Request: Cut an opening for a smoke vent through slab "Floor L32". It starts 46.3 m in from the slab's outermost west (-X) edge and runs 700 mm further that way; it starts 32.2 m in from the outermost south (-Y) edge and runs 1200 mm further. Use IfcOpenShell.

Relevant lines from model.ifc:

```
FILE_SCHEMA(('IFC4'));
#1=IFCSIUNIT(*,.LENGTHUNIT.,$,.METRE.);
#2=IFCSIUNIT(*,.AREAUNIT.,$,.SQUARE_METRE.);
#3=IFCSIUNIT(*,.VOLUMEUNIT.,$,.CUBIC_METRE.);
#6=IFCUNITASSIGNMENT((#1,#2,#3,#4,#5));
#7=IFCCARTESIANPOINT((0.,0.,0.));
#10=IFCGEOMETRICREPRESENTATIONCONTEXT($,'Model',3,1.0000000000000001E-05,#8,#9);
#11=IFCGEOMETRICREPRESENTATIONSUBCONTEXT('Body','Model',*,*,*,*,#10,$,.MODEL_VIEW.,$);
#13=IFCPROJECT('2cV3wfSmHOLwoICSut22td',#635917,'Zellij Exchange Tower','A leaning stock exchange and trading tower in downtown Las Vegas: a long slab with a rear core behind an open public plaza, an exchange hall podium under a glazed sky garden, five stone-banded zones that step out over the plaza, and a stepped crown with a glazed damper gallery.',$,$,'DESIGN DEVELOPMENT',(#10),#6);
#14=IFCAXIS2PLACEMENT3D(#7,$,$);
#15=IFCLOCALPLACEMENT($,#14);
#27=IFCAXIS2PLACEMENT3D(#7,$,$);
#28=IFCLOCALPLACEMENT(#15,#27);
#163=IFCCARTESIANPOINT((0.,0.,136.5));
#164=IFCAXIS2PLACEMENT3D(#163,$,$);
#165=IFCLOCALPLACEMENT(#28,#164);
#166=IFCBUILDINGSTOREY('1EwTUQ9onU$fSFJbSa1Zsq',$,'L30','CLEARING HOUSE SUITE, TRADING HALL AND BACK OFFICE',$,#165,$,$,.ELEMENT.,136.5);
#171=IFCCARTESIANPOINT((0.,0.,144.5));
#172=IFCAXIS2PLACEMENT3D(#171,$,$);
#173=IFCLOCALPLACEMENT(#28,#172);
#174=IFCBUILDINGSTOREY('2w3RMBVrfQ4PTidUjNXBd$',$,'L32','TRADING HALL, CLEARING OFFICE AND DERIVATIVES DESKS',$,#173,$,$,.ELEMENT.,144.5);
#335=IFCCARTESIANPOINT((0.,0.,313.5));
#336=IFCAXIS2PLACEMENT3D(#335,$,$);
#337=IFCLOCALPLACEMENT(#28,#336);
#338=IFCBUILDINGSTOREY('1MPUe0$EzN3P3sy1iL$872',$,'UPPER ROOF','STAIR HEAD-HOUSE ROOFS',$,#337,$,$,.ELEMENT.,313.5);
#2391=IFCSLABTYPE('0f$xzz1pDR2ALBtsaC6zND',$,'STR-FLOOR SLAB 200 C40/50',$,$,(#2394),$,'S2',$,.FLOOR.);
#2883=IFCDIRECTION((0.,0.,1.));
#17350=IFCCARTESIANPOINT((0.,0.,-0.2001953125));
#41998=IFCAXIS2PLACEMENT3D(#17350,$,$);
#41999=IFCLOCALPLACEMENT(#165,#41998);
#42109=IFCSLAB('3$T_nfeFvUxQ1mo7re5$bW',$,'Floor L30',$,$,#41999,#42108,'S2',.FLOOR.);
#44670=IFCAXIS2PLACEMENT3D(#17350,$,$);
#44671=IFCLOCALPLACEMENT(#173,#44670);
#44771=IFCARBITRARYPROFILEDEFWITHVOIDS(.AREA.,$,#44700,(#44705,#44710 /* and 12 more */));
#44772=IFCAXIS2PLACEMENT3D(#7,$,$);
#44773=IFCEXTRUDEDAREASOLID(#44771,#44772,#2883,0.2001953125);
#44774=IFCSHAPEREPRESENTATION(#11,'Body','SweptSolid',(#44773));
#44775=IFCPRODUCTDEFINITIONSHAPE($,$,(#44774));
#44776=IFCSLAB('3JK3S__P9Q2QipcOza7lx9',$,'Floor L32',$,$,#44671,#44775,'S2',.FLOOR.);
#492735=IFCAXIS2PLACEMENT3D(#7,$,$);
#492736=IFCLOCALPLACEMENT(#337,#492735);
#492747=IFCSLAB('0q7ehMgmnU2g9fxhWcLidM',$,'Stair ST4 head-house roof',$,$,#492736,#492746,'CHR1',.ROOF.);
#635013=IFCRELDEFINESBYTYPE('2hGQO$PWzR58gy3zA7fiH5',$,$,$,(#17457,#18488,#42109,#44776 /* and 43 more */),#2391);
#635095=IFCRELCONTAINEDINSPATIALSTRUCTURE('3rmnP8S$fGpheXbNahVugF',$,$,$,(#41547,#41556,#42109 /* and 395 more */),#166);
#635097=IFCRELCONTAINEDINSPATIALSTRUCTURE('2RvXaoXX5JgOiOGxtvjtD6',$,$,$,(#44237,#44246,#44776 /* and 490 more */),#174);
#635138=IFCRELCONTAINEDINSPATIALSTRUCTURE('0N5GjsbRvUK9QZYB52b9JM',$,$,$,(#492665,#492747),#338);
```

```python
import numpy as np
import ifcopenshell
import ifcopenshell.api.feature
import ifcopenshell.api.geometry
import ifcopenshell.api.root
import ifcopenshell.geom
import ifcopenshell.util.placement
import ifcopenshell.util.representation
import ifcopenshell.util.shape
import ifcopenshell.util.unit

model = ifcopenshell.open("model.ifc")
unit_scale = ifcopenshell.util.unit.calculate_unit_scale(model)
settings = ifcopenshell.geom.settings()


def volume(element):
    """Net volume in cubic metres, openings subtracted."""
    shape = ifcopenshell.geom.create_shape(settings, element)
    return ifcopenshell.util.shape.get_volume(shape.geometry)


slab = model.by_guid("3JK3S__P9Q2QipcOza7lx9")
before = volume(slab)

# Extent in the slab's own axes, in metres. The edges named are its -X and -Y sides.
slab_shape = ifcopenshell.geom.create_shape(settings, slab)
vertices = ifcopenshell.util.shape.get_vertices(slab_shape.geometry)
x_min, y_min, bottom = vertices.min(axis=0)
top = vertices[:, 2].max()

opening = ifcopenshell.api.root.create_entity(model, ifc_class="IfcOpeningElement", name="Smoke vent opening", predefined_type="OPENING")
context = ifcopenshell.util.representation.get_context(model, "Model", "Body", "MODEL_VIEW")
width, depth = 0.7, 1.2
outline = [(0.0, 0.0), (width, 0.0), (width, depth), (0.0, depth), (0.0, 0.0)]
# Overshoot both faces by 50 mm so the cut is clean.
shape = ifcopenshell.api.geometry.add_slab_representation(
    model, context=context, depth=top - bottom + 0.1, polyline=outline
)
ifcopenshell.api.geometry.assign_representation(model, product=opening, representation=shape)

matrix = ifcopenshell.util.placement.get_local_placement(slab.ObjectPlacement)
matrix[:, 3] = matrix @ np.append(np.array([x_min + 46.3, y_min + 32.2, bottom - 0.05]) / unit_scale, 1.0)
ifcopenshell.api.geometry.edit_object_placement(model, product=opening, matrix=matrix, is_si=False)
ifcopenshell.api.feature.add_feature(model, feature=opening, element=slab)

after = volume(slab)

print(f"slab volume {before:.3f} -> {after:.3f} m3")

model.write("model-out.ifc")
```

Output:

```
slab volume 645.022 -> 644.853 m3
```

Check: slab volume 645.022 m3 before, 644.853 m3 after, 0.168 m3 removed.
